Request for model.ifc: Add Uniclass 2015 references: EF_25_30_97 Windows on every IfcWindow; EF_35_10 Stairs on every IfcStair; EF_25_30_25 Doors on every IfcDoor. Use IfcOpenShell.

First a look at what the model holds.

```python
import ifcopenshell

model = ifcopenshell.open("model.ifc")
print(model.schema)
print("classifications:", [c.Name for c in model.by_type("IfcClassification")])
for ifc_class in ("IfcDoor", "IfcRoof", "IfcStair", "IfcWall", "IfcWindow"):
    print(ifc_class, len(model.by_type(ifc_class)))
```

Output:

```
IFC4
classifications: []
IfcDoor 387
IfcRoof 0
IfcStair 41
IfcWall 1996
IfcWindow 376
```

```python
import ifcopenshell
import ifcopenshell.api.classification

model = ifcopenshell.open("model.ifc")

system = ifcopenshell.api.classification.add_classification(model, classification="Uniclass 2015")

codes = {
    "IfcWindow": ("EF_25_30_97", "Windows"),
    "IfcStair": ("EF_35_10", "Stairs"),
    "IfcDoor": ("EF_25_30_25", "Doors"),
}
for ifc_class, (code, name) in codes.items():
    products = model.by_type(ifc_class)
    ifcopenshell.api.classification.add_reference(
        model, products=products, classification=system, identification=code, name=name
    )
    print(code, len(products))

model.write("model_rev.ifc")
```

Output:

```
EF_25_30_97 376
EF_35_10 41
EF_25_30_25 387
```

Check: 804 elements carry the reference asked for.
